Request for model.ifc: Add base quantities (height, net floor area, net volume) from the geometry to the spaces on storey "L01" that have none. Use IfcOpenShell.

First a look at what the model holds.

```python
import ifcopenshell
import ifcopenshell.util.element
import ifcopenshell.util.unit

model = ifcopenshell.open("model.ifc")
print(model.schema)
for unit_type in ("LENGTHUNIT", "AREAUNIT", "VOLUMEUNIT"):
    print(unit_type, ifcopenshell.util.unit.calculate_unit_scale(model, unit_type))
storey = next(s for s in model.by_type("IfcBuildingStorey") if s.Name == "L01")
spaces = [e for e in ifcopenshell.util.element.get_decomposition(storey) if e.is_a("IfcSpace")]
for e in sorted(spaces, key=lambda e: e.id()):
    print(e.id(), e.is_a(), e.Name, list(ifcopenshell.util.element.get_psets(e, qtos_only=True)), sep=" | ")
```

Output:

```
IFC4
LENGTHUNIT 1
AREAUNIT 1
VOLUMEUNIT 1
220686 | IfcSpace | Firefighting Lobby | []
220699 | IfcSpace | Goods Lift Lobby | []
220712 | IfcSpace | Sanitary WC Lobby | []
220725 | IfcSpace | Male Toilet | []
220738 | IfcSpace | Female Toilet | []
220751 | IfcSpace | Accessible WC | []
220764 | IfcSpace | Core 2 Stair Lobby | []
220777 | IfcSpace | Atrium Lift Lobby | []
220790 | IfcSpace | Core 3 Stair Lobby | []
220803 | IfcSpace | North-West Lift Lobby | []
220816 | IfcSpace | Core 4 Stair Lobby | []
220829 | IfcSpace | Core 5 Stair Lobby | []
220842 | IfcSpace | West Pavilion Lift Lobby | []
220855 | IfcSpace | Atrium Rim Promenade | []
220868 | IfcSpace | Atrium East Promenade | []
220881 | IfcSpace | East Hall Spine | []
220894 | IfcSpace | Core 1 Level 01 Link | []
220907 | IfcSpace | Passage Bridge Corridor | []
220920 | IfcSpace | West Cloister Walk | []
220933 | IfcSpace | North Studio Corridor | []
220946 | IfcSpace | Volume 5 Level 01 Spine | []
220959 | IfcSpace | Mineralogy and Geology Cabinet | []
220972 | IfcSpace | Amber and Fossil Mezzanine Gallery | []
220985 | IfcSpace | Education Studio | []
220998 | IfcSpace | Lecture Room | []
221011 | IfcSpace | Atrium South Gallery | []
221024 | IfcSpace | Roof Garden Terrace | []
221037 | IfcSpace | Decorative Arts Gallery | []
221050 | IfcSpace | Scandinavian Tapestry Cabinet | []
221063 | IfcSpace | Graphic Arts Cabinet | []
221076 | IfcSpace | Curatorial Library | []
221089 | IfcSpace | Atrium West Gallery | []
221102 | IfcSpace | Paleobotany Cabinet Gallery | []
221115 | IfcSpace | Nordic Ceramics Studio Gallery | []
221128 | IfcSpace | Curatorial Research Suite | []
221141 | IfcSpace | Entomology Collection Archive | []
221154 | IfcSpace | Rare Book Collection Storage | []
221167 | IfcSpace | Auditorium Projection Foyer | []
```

```python
import ifcopenshell
import ifcopenshell.api.pset
import ifcopenshell.geom
import ifcopenshell.util.element
import ifcopenshell.util.shape
import ifcopenshell.util.unit

model = ifcopenshell.open("model.ifc")
unit_scale = ifcopenshell.util.unit.calculate_unit_scale(model)
area_scale = ifcopenshell.util.unit.calculate_unit_scale(model, "AREAUNIT")
volume_scale = ifcopenshell.util.unit.calculate_unit_scale(model, "VOLUMEUNIT")
settings = ifcopenshell.geom.settings()

storey = next(s for s in model.by_type("IfcBuildingStorey") if s.Name == "L01")
spaces = [e for e in ifcopenshell.util.element.get_decomposition(storey) if e.is_a("IfcSpace")]

for e in sorted(spaces, key=lambda e: e.id()):
    if ifcopenshell.util.element.get_psets(e, qtos_only=True, should_inherit=False):
        continue
    # Geometry comes back in metres, in the element's own axes.
    shape = ifcopenshell.geom.create_shape(settings, e)
    values = {
        "Height": ifcopenshell.util.shape.get_z(shape.geometry) / unit_scale,
        "NetFloorArea": ifcopenshell.util.shape.get_footprint_area(shape.geometry) / area_scale,
        "NetVolume": ifcopenshell.util.shape.get_volume(shape.geometry) / volume_scale,
    }
    qto = ifcopenshell.api.pset.add_qto(model, product=e, name="Qto_SpaceBaseQuantities")
    ifcopenshell.api.pset.edit_qto(model, qto=qto, properties=values)
    print(e.id(), {k: round(v, 3) for k, v in values.items()})

model.write("model_rev.ifc")
```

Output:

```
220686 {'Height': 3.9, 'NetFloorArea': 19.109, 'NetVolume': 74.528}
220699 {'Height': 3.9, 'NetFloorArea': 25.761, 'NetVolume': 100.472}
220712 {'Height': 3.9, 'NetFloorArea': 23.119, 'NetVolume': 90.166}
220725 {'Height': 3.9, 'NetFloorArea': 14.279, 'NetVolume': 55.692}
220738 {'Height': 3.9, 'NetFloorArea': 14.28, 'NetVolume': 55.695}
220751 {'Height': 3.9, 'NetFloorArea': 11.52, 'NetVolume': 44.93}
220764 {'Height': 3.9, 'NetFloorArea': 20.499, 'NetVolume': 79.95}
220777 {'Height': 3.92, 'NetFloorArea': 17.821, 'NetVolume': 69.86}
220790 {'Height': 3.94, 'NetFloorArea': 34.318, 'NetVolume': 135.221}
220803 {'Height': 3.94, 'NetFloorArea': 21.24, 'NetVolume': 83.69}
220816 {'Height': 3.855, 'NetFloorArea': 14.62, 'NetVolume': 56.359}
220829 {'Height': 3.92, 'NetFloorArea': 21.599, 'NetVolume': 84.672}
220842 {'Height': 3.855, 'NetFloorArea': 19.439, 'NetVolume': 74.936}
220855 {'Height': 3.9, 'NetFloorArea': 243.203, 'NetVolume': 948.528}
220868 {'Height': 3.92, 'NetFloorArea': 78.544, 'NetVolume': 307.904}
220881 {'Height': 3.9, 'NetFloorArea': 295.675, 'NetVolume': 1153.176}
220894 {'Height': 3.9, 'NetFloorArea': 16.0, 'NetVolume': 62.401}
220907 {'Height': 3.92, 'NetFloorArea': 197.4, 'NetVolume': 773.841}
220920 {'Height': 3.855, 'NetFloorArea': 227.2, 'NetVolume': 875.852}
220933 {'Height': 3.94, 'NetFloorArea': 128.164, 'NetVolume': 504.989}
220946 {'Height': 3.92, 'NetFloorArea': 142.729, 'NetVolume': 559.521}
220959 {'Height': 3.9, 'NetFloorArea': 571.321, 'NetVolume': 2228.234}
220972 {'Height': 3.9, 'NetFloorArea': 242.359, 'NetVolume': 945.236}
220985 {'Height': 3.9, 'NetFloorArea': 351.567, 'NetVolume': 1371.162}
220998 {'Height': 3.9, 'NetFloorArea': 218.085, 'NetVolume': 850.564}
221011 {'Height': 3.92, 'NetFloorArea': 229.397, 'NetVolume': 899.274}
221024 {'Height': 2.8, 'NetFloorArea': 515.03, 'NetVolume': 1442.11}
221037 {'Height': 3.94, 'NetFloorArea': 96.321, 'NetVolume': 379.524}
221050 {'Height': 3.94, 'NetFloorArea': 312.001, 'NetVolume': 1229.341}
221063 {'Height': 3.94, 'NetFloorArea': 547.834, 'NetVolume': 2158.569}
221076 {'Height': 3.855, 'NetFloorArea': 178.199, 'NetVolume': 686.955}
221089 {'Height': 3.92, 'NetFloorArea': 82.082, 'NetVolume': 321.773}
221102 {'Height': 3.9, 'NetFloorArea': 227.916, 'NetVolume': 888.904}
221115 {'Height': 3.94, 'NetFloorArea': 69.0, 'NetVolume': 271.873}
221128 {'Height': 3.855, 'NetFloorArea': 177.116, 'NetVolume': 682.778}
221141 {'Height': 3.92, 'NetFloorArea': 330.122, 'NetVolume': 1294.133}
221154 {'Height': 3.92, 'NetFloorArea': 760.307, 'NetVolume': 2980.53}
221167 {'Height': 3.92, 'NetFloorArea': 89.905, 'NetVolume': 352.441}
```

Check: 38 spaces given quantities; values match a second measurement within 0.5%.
